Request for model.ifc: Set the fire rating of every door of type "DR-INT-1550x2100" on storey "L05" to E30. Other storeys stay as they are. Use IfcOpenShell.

First a look at what the model holds.

```python
import ifcopenshell
import ifcopenshell.util.element

model = ifcopenshell.open("model.ifc")
print(model.schema)
storey = next(s for s in model.by_type("IfcBuildingStorey") if s.Name == "L05")
doors = [e for e in ifcopenshell.util.element.get_decomposition(storey) if e.is_a("IfcDoor")]
seen = {}
for e in doors:
    element_type = ifcopenshell.util.element.get_type(e)
    key = (element_type.Name if element_type != e and element_type else None, ifcopenshell.util.element.get_pset(e, "Pset_DoorCommon", "FireRating"))
    seen[key] = seen.get(key, 0) + 1
for (name, value), count in sorted(seen.items(), key=str):
    print(count, "x", name, "|", value)
```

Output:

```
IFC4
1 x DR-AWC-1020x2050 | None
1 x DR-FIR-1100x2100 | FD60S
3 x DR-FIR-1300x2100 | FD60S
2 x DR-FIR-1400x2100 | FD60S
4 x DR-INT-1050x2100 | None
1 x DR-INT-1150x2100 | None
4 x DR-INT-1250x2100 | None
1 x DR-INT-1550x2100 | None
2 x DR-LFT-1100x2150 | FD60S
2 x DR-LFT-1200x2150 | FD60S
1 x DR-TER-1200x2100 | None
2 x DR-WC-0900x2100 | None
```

```python
import ifcopenshell
import ifcopenshell.api.pset
import ifcopenshell.util.element

model = ifcopenshell.open("model.ifc")

storey = next(s for s in model.by_type("IfcBuildingStorey") if s.Name == "L05")
doors = [e for e in ifcopenshell.util.element.get_decomposition(storey) if e.is_a("IfcDoor")]

count = 0
for e in doors:
    element_type = ifcopenshell.util.element.get_type(e)
    if element_type in (None, e) or element_type.Name != "DR-INT-1550x2100":
        continue
    # add_pset returns the element's existing set when there is one.
    pset = ifcopenshell.api.pset.add_pset(model, product=e, name="Pset_DoorCommon")
    ifcopenshell.api.pset.edit_pset(model, pset=pset, properties={"FireRating": "E30"})
    count += 1

print(count, "doors updated")

model.write("model_v2.ifc")
```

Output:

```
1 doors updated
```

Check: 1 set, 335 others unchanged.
